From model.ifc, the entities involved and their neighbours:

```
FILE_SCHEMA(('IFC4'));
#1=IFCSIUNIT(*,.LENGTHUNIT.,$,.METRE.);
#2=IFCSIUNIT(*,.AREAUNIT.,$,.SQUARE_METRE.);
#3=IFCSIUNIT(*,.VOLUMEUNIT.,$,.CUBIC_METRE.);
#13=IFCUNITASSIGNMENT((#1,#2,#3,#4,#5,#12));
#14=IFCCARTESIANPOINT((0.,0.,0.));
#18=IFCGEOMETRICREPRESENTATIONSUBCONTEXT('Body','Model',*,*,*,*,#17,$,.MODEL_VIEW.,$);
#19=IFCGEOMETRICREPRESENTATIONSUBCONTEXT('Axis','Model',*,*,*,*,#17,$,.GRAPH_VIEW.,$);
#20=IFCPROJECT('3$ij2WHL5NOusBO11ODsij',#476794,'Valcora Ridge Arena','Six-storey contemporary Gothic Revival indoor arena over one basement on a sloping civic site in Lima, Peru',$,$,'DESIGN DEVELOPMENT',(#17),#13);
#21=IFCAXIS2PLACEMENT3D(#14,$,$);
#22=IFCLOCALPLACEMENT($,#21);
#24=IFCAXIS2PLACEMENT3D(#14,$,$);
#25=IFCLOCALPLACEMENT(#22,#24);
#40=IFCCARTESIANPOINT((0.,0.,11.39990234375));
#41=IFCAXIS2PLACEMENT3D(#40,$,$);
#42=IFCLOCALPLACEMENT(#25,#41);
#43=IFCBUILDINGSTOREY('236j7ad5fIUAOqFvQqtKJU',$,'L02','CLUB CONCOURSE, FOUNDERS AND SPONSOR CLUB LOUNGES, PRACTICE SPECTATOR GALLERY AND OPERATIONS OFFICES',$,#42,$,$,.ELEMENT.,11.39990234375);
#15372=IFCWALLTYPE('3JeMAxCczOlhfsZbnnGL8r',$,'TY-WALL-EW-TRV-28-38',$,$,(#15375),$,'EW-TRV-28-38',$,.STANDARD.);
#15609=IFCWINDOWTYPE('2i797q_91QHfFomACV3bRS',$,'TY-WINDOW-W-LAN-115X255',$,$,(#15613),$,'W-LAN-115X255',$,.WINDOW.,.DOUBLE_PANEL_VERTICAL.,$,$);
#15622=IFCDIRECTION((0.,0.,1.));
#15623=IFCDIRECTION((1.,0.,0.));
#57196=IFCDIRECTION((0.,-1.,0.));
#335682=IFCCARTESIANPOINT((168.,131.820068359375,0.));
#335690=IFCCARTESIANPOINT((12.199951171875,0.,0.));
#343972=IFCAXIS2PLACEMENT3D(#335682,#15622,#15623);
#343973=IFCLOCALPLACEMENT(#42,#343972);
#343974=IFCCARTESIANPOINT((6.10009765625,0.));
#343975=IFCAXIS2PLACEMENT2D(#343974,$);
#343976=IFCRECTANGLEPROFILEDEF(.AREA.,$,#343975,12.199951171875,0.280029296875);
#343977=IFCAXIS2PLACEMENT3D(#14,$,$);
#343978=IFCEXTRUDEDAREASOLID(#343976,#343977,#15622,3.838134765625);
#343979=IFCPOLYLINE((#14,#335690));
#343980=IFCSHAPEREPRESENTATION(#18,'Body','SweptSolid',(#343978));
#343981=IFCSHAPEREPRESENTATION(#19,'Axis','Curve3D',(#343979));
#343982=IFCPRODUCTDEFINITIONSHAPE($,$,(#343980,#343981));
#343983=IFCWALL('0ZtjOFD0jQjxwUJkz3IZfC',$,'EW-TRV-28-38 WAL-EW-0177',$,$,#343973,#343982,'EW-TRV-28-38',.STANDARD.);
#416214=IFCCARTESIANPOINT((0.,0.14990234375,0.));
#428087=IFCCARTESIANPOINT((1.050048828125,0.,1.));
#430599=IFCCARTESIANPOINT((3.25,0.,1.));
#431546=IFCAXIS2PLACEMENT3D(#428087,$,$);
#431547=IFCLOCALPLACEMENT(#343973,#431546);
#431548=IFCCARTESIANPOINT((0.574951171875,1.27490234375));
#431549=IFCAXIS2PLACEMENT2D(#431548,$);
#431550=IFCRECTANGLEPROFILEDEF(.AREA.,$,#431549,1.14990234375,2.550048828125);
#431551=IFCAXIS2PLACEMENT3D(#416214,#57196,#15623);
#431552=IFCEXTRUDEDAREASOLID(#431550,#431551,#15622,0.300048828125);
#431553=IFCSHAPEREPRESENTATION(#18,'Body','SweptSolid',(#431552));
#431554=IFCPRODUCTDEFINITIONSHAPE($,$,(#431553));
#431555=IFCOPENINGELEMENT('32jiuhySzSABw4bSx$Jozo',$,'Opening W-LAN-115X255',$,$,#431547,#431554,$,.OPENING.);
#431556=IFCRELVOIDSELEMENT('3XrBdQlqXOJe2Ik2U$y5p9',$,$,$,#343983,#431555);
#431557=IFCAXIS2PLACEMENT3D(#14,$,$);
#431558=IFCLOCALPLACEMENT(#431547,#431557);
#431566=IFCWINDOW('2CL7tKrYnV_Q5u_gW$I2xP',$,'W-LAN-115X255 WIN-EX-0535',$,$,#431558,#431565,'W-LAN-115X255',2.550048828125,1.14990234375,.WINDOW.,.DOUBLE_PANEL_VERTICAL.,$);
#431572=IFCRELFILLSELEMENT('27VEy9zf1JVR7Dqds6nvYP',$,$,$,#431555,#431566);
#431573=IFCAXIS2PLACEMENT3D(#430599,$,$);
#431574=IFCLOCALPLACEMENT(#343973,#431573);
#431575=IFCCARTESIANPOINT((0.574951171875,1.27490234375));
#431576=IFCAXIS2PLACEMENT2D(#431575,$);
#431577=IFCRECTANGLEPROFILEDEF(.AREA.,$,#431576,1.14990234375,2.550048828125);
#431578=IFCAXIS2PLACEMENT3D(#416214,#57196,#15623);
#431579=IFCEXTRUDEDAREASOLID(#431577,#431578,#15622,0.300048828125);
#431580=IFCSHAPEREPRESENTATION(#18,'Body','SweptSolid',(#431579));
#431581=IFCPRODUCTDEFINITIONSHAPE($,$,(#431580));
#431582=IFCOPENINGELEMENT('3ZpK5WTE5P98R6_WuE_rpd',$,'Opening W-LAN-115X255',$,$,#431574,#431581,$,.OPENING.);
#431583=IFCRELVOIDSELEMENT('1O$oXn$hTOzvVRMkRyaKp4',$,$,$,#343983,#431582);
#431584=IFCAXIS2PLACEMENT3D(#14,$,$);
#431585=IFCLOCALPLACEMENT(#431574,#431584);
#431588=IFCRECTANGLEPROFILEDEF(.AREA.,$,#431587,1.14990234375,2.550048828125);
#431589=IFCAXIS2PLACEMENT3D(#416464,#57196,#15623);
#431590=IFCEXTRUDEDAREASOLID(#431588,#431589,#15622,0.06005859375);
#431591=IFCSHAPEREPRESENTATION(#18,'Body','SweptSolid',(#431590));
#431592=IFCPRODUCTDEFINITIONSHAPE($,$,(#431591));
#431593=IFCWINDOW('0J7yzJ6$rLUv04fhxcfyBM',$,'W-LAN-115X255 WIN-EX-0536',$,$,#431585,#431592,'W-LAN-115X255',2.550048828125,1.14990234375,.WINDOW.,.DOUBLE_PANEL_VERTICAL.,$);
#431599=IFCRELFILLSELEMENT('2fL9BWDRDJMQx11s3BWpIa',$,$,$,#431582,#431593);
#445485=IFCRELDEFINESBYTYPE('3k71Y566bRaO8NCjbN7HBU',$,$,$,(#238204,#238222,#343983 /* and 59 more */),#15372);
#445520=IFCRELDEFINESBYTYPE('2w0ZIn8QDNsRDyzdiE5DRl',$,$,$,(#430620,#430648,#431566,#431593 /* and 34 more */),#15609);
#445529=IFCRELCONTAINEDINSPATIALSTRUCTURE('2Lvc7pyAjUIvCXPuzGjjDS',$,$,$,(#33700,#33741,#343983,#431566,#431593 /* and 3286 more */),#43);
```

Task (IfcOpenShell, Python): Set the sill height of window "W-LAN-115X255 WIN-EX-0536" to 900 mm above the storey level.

```python
import numpy as np
import ifcopenshell
import ifcopenshell.api.geometry
import ifcopenshell.geom
import ifcopenshell.util.element
import ifcopenshell.util.placement
import ifcopenshell.util.shape
import ifcopenshell.util.unit

model = ifcopenshell.open("model.ifc")
unit_scale = ifcopenshell.util.unit.calculate_unit_scale(model)

window = model.by_guid("0J7yzJ6$rLUv04fhxcfyBM")
opening = window.FillsVoids[0].RelatingOpeningElement
storey = ifcopenshell.util.element.get_container(window, ifc_class="IfcBuildingStorey")
level = ifcopenshell.util.placement.get_local_placement(storey.ObjectPlacement)[2, 3]

# The opening's origin need not be at the sill, so measure its lowest point.
shape = ifcopenshell.geom.create_shape(ifcopenshell.geom.settings(), opening)
bottom = ifcopenshell.util.shape.get_shape_bottom_elevation(shape, shape.geometry) / unit_scale
dz = level + 0.9 - bottom

shift = np.array([0.0, 0.0, dz])
# The window is placed relative to its opening, so it follows when the opening moves.
matrix = ifcopenshell.util.placement.get_local_placement(opening.ObjectPlacement)
matrix[:3, 3] += shift
ifcopenshell.api.geometry.edit_object_placement(
    model, product=opening, matrix=matrix, is_si=False, should_transform_children=True
)

print(f"moved by {dz * unit_scale:+.3f} m")

model.write("model_rev.ifc")
```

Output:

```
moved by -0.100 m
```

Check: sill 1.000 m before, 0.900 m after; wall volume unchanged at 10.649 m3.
